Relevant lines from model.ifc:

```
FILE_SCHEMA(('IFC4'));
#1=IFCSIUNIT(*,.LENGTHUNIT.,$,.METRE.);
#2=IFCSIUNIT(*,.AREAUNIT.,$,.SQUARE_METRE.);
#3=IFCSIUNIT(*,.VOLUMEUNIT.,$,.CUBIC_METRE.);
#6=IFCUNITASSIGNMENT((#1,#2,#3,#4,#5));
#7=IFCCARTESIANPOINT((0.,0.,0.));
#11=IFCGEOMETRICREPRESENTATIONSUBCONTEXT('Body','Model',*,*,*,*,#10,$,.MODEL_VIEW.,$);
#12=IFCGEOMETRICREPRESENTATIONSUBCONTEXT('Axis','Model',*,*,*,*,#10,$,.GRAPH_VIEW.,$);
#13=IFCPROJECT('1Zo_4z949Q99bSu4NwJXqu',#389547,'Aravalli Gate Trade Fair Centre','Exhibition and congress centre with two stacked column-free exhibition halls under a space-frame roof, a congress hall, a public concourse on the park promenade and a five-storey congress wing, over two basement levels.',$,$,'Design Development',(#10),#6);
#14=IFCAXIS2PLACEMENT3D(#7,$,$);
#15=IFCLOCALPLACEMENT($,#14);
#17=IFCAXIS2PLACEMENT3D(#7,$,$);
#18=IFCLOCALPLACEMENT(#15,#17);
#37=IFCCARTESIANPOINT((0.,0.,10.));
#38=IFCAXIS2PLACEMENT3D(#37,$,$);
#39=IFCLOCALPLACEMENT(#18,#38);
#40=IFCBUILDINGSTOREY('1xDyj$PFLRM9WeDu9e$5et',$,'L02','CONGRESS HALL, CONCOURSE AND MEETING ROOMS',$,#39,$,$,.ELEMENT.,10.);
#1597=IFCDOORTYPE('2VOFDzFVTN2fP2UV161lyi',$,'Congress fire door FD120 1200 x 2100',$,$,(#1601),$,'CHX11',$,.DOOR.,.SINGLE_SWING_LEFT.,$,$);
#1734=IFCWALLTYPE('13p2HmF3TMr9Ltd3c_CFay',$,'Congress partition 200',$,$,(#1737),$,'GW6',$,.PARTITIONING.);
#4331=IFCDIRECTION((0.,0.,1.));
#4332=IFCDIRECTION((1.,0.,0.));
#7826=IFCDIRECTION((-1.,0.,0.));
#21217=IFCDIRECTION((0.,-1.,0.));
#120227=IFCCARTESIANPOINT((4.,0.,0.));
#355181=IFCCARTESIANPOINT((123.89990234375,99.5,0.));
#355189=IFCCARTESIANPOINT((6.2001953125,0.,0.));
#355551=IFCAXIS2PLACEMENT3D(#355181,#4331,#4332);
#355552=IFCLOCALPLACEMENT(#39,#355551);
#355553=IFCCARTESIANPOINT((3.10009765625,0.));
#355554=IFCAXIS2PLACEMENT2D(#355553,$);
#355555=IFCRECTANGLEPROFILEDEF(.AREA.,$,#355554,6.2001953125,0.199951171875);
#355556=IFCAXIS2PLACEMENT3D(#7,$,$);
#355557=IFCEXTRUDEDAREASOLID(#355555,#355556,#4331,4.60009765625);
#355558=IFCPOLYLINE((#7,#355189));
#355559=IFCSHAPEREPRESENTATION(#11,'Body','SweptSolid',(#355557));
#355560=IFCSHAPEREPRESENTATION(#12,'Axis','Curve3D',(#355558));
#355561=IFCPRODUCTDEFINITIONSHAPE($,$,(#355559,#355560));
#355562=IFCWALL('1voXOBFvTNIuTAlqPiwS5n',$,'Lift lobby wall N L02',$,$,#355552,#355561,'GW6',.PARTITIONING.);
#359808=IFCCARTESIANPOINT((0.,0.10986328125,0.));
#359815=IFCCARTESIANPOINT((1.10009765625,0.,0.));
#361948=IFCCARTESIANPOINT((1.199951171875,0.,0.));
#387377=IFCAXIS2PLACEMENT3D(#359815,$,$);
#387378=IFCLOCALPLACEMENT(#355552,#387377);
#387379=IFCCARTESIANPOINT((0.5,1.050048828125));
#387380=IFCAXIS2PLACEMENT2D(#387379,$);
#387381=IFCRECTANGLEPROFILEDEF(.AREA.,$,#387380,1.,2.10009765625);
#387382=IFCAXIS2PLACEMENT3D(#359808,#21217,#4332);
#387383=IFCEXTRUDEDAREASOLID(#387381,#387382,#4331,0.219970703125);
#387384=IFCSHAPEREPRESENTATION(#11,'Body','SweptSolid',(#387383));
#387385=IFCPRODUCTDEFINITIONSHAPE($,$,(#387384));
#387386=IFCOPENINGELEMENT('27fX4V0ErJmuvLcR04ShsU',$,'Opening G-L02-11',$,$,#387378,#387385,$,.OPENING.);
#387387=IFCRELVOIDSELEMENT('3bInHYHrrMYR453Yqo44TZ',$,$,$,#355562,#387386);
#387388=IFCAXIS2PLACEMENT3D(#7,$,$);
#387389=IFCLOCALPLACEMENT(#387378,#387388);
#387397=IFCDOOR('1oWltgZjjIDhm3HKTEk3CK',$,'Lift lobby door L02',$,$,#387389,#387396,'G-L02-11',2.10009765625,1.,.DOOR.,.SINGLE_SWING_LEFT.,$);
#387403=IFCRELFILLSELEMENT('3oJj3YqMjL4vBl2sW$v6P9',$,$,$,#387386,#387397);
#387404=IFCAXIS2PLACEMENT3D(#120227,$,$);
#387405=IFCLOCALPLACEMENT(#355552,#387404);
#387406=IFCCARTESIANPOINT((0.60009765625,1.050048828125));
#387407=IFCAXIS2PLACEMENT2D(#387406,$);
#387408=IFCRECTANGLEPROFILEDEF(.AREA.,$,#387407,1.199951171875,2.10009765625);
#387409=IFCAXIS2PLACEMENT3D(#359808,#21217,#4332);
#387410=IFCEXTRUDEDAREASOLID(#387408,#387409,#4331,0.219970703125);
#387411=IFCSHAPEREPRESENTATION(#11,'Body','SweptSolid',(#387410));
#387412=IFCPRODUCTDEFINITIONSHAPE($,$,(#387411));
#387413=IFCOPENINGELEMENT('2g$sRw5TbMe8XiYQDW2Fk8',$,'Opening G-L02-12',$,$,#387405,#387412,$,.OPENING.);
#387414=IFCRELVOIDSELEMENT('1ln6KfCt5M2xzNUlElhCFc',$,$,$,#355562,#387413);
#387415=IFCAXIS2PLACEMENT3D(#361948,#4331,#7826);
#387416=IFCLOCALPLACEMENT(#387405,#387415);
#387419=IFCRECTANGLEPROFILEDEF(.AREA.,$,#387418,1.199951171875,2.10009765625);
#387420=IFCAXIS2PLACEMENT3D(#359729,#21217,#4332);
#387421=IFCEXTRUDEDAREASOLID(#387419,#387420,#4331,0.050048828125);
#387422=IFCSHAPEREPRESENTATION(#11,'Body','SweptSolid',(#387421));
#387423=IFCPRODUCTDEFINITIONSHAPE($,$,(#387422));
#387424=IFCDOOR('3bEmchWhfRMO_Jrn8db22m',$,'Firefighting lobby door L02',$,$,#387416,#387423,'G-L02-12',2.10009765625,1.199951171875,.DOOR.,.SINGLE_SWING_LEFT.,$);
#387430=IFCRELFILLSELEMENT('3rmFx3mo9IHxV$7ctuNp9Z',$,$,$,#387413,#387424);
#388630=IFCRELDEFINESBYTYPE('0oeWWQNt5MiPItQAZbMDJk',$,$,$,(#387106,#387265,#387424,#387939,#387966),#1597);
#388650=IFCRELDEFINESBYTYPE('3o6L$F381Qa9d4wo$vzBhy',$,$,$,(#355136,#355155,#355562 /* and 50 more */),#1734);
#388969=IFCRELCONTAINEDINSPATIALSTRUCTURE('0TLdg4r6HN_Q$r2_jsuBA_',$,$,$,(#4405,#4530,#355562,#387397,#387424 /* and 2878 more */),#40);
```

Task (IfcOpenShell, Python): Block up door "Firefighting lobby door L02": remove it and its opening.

```python
import ifcopenshell
import ifcopenshell.api.feature
import ifcopenshell.api.root
import ifcopenshell.geom
import ifcopenshell.util.shape

model = ifcopenshell.open("model.ifc")
settings = ifcopenshell.geom.settings()


def volume(element):
    """Net volume in cubic metres, openings subtracted."""
    shape = ifcopenshell.geom.create_shape(settings, element)
    return ifcopenshell.util.shape.get_volume(shape.geometry)


door = model.by_guid("3bEmchWhfRMO_Jrn8db22m")
opening = door.FillsVoids[0].RelatingOpeningElement
wall = opening.VoidsElements[0].RelatingBuildingElement
before = volume(wall)

ifcopenshell.api.root.remove_product(model, product=door)
ifcopenshell.api.feature.remove_feature(model, feature=opening)

after = volume(wall)

print(f"wall volume {before:.3f} -> {after:.3f} m3")

model.write("model_edited.ifc")
```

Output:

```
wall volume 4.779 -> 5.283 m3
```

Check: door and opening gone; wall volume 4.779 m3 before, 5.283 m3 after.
